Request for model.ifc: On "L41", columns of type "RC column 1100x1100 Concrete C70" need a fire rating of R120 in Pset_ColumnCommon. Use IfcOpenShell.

First a look at what the model holds.

```python
import ifcopenshell
import ifcopenshell.util.element

model = ifcopenshell.open("model.ifc")
print(model.schema)
storey = next(s for s in model.by_type("IfcBuildingStorey") if s.Name == "L41")
columns = [e for e in ifcopenshell.util.element.get_decomposition(storey) if e.is_a("IfcColumn")]
seen = {}
for e in columns:
    element_type = ifcopenshell.util.element.get_type(e)
    key = (element_type.Name if element_type != e and element_type else None, ifcopenshell.util.element.get_pset(e, "Pset_ColumnCommon", "FireRating"))
    seen[key] = seen.get(key, 0) + 1
for (name, value), count in sorted(seen.items(), key=str):
    print(count, "x", name, "|", value)
```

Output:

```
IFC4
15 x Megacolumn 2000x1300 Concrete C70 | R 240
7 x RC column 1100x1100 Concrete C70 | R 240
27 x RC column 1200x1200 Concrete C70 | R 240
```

```python
import ifcopenshell
import ifcopenshell.api.pset
import ifcopenshell.util.element

model = ifcopenshell.open("model.ifc")

storey = next(s for s in model.by_type("IfcBuildingStorey") if s.Name == "L41")
columns = [e for e in ifcopenshell.util.element.get_decomposition(storey) if e.is_a("IfcColumn")]

count = 0
for e in columns:
    element_type = ifcopenshell.util.element.get_type(e)
    if element_type in (None, e) or element_type.Name != "RC column 1100x1100 Concrete C70":
        continue
    found = ifcopenshell.util.element.get_pset(e, "Pset_ColumnCommon", should_inherit=False)
    if found:
        pset = model.by_id(found["id"])
        if len(ifcopenshell.util.element.get_elements_by_pset(pset)) > 1:
            pset = ifcopenshell.api.pset.unshare_pset(model, products=[e], pset=pset)[0]
    else:
        pset = ifcopenshell.api.pset.add_pset(model, product=e, name="Pset_ColumnCommon")
    ifcopenshell.api.pset.edit_pset(model, pset=pset, properties={"FireRating": "R120"})
    count += 1

print(count, "columns updated")

model.write("model_rev.ifc")
```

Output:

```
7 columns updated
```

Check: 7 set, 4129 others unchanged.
